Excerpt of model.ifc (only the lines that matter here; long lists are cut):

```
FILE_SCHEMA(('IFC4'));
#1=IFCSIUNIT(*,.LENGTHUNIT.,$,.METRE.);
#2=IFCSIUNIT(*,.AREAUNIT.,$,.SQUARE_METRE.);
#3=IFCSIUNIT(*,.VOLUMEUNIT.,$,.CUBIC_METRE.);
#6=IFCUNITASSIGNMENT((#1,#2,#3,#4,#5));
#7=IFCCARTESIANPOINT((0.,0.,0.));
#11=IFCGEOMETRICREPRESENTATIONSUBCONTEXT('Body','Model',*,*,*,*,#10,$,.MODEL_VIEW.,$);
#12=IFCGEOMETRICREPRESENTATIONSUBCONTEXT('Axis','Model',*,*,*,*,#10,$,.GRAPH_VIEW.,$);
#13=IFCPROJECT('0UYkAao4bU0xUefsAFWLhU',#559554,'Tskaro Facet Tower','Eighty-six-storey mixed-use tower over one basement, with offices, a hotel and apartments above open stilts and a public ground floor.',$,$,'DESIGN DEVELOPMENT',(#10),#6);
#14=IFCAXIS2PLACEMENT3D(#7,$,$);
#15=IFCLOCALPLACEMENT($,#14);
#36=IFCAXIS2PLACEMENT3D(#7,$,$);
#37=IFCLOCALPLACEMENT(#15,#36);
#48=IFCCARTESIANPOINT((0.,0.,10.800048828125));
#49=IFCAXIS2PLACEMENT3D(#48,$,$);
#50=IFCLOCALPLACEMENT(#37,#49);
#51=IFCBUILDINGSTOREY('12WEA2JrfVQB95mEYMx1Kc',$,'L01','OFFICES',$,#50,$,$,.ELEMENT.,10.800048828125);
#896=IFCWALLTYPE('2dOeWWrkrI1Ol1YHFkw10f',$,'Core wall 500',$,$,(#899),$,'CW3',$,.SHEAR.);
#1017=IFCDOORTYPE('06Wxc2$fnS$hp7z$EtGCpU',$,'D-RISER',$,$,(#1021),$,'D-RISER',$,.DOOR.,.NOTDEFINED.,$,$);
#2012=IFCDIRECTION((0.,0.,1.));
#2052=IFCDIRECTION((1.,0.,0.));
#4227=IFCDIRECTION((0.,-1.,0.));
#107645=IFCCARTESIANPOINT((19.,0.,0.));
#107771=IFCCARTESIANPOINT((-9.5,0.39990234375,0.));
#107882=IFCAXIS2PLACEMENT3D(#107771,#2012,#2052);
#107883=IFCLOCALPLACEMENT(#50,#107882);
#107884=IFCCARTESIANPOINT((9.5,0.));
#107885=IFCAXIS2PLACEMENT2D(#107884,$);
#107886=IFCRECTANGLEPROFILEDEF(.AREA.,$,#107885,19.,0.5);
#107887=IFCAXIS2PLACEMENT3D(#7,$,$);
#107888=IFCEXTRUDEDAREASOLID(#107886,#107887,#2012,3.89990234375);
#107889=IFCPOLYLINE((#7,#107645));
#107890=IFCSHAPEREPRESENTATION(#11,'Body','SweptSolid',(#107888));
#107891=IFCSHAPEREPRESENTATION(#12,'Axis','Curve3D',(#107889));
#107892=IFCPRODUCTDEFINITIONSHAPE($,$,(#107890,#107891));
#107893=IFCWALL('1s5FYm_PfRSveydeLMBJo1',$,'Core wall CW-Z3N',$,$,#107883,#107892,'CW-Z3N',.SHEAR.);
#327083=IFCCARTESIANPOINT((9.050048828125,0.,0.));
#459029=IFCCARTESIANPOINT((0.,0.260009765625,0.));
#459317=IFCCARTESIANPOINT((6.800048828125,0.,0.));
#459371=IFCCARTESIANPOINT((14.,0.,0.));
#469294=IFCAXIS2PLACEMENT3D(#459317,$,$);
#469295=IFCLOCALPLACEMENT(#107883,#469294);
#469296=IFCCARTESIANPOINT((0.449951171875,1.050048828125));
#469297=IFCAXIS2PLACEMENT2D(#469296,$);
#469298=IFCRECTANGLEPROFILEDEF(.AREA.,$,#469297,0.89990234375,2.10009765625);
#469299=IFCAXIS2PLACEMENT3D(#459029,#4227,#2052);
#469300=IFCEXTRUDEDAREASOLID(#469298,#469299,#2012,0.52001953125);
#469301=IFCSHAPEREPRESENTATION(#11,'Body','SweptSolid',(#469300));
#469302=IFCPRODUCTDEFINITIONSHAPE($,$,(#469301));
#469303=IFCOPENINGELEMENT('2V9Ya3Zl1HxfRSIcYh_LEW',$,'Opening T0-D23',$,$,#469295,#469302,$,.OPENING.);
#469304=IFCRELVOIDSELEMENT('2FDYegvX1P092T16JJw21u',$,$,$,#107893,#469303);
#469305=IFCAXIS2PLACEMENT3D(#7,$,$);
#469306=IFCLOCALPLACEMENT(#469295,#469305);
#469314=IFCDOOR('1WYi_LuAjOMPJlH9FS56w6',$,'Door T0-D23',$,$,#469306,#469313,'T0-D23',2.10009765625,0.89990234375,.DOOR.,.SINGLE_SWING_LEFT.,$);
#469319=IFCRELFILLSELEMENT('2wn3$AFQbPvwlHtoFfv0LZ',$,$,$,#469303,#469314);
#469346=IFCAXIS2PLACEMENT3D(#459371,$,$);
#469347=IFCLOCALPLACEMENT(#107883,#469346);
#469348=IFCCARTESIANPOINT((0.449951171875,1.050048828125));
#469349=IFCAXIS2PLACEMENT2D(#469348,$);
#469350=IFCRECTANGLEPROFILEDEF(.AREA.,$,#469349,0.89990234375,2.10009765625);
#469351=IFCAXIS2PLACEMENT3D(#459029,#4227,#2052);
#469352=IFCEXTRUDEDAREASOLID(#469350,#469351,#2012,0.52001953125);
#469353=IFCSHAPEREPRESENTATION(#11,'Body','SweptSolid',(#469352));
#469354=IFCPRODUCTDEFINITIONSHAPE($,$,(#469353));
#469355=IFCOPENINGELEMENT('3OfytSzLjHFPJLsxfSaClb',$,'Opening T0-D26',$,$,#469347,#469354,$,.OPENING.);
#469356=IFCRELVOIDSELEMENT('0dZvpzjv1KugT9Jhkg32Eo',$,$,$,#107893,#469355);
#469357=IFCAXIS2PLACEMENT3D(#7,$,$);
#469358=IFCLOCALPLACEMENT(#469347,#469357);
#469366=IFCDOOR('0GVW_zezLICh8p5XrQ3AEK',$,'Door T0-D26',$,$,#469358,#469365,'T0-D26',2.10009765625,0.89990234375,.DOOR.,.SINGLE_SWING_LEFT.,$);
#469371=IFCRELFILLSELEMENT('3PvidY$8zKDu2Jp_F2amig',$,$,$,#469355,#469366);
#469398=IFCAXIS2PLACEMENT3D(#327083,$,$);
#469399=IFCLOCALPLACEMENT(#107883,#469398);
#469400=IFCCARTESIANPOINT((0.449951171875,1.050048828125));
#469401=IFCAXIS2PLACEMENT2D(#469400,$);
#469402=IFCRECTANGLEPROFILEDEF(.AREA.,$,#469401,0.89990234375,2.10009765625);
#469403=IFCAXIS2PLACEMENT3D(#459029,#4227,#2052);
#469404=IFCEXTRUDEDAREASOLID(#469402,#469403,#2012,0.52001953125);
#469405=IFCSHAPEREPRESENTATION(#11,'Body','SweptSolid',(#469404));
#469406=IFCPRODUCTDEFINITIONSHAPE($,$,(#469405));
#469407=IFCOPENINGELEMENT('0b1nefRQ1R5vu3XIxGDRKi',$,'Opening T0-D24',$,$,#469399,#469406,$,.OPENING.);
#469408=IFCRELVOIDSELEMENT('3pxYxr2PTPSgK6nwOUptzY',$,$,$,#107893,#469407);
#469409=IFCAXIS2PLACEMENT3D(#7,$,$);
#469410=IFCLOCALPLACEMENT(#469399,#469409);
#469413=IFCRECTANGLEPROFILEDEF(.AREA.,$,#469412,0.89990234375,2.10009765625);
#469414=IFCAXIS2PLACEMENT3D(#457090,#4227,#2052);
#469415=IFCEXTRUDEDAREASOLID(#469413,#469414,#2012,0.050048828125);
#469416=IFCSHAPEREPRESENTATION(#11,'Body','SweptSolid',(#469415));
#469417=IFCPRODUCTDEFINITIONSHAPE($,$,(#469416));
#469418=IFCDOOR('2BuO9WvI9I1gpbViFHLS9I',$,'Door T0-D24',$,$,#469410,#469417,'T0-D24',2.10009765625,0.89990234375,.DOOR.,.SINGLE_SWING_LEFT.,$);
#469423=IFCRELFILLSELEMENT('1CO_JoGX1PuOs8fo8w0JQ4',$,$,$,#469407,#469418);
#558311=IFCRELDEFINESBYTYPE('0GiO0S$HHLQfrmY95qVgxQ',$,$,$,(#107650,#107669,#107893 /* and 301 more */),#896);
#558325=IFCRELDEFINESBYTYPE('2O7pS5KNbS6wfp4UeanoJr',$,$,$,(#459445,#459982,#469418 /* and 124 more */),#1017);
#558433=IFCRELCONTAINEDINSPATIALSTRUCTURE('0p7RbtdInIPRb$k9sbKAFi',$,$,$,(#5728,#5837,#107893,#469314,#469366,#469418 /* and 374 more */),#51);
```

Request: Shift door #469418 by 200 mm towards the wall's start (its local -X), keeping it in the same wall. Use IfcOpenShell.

```python
import ifcopenshell
import ifcopenshell.api.geometry
import ifcopenshell.util.placement

model = ifcopenshell.open("model.ifc")

door = model.by_guid("2BuO9WvI9I1gpbViFHLS9I")
opening = door.FillsVoids[0].RelatingOpeningElement
wall = opening.VoidsElements[0].RelatingBuildingElement

wall_matrix = ifcopenshell.util.placement.get_local_placement(wall.ObjectPlacement)
shift = wall_matrix[:3, 0] * -0.2
before = ifcopenshell.util.placement.get_local_placement(door.ObjectPlacement)[:3, 3].copy()

# The door is placed relative to its opening, so it follows when the opening moves.
matrix = ifcopenshell.util.placement.get_local_placement(opening.ObjectPlacement)
matrix[:3, 3] += shift
ifcopenshell.api.geometry.edit_object_placement(
    model, product=opening, matrix=matrix, is_si=False, should_transform_children=True
)

after = ifcopenshell.util.placement.get_local_placement(door.ObjectPlacement)[:3, 3]
print("door moved by", (after - before).round(3) + 0.0)

model.write("model_edited.ifc")
```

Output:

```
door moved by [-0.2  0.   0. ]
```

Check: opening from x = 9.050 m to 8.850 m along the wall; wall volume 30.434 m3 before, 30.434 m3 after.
